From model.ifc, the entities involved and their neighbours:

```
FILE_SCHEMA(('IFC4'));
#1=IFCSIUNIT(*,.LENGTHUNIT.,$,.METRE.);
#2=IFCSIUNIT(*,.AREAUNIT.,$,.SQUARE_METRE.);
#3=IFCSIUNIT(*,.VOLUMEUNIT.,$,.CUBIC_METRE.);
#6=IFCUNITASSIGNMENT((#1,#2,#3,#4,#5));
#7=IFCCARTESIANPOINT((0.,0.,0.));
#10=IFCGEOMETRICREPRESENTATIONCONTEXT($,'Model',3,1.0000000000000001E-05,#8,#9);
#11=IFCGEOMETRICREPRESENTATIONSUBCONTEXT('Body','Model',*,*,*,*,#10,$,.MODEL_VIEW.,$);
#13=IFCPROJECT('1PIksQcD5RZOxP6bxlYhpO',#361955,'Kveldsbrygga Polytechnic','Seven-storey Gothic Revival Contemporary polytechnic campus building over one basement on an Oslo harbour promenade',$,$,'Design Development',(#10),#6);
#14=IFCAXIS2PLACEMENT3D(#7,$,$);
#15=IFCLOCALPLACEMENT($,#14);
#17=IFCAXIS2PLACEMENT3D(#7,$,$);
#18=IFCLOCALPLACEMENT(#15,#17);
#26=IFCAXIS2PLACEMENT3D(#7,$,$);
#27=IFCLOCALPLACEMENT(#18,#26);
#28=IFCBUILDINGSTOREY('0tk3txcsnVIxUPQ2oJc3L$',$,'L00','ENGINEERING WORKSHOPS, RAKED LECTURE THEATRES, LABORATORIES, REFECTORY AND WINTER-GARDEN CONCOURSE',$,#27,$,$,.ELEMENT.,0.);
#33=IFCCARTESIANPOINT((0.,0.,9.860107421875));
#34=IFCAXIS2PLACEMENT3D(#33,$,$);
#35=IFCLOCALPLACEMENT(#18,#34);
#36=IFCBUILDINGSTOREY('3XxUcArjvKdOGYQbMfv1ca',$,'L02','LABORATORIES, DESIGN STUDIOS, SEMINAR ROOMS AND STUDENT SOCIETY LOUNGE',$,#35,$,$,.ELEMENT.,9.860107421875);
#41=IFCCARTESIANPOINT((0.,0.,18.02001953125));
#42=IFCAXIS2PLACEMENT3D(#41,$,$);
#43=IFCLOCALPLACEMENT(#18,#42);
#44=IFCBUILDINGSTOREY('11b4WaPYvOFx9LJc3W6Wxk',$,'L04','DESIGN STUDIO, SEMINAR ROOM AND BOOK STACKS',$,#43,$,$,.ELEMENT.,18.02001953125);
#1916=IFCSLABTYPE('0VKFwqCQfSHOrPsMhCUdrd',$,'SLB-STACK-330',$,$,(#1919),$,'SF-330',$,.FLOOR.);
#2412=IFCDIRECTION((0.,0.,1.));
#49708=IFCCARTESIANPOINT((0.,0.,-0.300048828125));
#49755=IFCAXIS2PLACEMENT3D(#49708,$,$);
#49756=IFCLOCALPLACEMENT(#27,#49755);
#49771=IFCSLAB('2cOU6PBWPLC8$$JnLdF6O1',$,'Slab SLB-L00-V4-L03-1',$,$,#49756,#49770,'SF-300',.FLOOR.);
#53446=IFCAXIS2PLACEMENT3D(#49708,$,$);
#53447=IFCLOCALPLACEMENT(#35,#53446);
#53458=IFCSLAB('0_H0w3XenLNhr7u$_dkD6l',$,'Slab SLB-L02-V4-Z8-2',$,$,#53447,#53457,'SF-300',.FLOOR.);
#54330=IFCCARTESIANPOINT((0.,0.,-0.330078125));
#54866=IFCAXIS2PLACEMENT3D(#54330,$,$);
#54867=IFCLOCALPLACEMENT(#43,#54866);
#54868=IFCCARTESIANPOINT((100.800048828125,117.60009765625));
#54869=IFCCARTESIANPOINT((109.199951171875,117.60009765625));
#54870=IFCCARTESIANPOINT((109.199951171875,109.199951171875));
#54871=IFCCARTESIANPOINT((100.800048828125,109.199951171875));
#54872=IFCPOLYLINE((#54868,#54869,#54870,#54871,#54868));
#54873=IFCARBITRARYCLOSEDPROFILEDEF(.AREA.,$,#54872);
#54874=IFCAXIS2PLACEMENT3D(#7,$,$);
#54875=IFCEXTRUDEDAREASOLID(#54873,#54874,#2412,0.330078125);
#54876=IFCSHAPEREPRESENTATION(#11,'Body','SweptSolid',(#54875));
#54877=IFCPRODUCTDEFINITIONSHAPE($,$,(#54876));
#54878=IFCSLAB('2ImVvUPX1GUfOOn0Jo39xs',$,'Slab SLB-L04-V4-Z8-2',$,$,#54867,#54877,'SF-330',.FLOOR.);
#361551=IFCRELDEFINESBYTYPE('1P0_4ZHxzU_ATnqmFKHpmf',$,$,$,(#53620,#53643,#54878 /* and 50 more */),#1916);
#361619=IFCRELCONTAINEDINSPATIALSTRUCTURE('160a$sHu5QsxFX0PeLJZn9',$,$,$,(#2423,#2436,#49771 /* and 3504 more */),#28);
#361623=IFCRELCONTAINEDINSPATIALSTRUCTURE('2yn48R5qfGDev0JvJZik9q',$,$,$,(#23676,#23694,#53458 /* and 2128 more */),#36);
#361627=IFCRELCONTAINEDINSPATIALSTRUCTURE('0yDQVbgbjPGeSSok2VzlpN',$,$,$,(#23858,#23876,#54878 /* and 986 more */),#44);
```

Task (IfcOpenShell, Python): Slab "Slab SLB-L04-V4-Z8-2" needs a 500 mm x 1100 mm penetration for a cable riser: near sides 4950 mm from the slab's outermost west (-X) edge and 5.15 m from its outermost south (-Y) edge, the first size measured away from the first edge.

```python
import numpy as np
import ifcopenshell
import ifcopenshell.api.feature
import ifcopenshell.api.geometry
import ifcopenshell.api.root
import ifcopenshell.geom
import ifcopenshell.util.placement
import ifcopenshell.util.representation
import ifcopenshell.util.shape
import ifcopenshell.util.unit

model = ifcopenshell.open("model.ifc")
unit_scale = ifcopenshell.util.unit.calculate_unit_scale(model)
settings = ifcopenshell.geom.settings()


def volume(element):
    """Net volume in cubic metres, openings subtracted."""
    shape = ifcopenshell.geom.create_shape(settings, element)
    return ifcopenshell.util.shape.get_volume(shape.geometry)


slab = model.by_guid("2ImVvUPX1GUfOOn0Jo39xs")
before = volume(slab)

# Extent in the slab's own axes, in metres. The edges named are its -X and -Y sides.
slab_shape = ifcopenshell.geom.create_shape(settings, slab)
vertices = ifcopenshell.util.shape.get_vertices(slab_shape.geometry)
x_min, y_min, bottom = vertices.min(axis=0)
top = vertices[:, 2].max()

opening = ifcopenshell.api.root.create_entity(model, ifc_class="IfcOpeningElement", name="Cable riser opening", predefined_type="OPENING")
context = ifcopenshell.util.representation.get_context(model, "Model", "Body", "MODEL_VIEW")
width, depth = 0.5, 1.1
outline = [(0.0, 0.0), (width, 0.0), (width, depth), (0.0, depth), (0.0, 0.0)]
# Overshoot both faces by 50 mm so the cut is clean.
shape = ifcopenshell.api.geometry.add_slab_representation(
    model, context=context, depth=top - bottom + 0.1, polyline=outline
)
ifcopenshell.api.geometry.assign_representation(model, product=opening, representation=shape)

matrix = ifcopenshell.util.placement.get_local_placement(slab.ObjectPlacement)
matrix[:, 3] = matrix @ np.append(np.array([x_min + 4.95, y_min + 5.15, bottom - 0.05]) / unit_scale, 1.0)
ifcopenshell.api.geometry.edit_object_placement(model, product=opening, matrix=matrix, is_si=False)
ifcopenshell.api.feature.add_feature(model, feature=opening, element=slab)

after = volume(slab)

print(f"slab volume {before:.3f} -> {after:.3f} m3")

model.write("model_edited.ifc")
```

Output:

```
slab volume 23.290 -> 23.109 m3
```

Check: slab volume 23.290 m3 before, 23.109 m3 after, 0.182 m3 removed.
